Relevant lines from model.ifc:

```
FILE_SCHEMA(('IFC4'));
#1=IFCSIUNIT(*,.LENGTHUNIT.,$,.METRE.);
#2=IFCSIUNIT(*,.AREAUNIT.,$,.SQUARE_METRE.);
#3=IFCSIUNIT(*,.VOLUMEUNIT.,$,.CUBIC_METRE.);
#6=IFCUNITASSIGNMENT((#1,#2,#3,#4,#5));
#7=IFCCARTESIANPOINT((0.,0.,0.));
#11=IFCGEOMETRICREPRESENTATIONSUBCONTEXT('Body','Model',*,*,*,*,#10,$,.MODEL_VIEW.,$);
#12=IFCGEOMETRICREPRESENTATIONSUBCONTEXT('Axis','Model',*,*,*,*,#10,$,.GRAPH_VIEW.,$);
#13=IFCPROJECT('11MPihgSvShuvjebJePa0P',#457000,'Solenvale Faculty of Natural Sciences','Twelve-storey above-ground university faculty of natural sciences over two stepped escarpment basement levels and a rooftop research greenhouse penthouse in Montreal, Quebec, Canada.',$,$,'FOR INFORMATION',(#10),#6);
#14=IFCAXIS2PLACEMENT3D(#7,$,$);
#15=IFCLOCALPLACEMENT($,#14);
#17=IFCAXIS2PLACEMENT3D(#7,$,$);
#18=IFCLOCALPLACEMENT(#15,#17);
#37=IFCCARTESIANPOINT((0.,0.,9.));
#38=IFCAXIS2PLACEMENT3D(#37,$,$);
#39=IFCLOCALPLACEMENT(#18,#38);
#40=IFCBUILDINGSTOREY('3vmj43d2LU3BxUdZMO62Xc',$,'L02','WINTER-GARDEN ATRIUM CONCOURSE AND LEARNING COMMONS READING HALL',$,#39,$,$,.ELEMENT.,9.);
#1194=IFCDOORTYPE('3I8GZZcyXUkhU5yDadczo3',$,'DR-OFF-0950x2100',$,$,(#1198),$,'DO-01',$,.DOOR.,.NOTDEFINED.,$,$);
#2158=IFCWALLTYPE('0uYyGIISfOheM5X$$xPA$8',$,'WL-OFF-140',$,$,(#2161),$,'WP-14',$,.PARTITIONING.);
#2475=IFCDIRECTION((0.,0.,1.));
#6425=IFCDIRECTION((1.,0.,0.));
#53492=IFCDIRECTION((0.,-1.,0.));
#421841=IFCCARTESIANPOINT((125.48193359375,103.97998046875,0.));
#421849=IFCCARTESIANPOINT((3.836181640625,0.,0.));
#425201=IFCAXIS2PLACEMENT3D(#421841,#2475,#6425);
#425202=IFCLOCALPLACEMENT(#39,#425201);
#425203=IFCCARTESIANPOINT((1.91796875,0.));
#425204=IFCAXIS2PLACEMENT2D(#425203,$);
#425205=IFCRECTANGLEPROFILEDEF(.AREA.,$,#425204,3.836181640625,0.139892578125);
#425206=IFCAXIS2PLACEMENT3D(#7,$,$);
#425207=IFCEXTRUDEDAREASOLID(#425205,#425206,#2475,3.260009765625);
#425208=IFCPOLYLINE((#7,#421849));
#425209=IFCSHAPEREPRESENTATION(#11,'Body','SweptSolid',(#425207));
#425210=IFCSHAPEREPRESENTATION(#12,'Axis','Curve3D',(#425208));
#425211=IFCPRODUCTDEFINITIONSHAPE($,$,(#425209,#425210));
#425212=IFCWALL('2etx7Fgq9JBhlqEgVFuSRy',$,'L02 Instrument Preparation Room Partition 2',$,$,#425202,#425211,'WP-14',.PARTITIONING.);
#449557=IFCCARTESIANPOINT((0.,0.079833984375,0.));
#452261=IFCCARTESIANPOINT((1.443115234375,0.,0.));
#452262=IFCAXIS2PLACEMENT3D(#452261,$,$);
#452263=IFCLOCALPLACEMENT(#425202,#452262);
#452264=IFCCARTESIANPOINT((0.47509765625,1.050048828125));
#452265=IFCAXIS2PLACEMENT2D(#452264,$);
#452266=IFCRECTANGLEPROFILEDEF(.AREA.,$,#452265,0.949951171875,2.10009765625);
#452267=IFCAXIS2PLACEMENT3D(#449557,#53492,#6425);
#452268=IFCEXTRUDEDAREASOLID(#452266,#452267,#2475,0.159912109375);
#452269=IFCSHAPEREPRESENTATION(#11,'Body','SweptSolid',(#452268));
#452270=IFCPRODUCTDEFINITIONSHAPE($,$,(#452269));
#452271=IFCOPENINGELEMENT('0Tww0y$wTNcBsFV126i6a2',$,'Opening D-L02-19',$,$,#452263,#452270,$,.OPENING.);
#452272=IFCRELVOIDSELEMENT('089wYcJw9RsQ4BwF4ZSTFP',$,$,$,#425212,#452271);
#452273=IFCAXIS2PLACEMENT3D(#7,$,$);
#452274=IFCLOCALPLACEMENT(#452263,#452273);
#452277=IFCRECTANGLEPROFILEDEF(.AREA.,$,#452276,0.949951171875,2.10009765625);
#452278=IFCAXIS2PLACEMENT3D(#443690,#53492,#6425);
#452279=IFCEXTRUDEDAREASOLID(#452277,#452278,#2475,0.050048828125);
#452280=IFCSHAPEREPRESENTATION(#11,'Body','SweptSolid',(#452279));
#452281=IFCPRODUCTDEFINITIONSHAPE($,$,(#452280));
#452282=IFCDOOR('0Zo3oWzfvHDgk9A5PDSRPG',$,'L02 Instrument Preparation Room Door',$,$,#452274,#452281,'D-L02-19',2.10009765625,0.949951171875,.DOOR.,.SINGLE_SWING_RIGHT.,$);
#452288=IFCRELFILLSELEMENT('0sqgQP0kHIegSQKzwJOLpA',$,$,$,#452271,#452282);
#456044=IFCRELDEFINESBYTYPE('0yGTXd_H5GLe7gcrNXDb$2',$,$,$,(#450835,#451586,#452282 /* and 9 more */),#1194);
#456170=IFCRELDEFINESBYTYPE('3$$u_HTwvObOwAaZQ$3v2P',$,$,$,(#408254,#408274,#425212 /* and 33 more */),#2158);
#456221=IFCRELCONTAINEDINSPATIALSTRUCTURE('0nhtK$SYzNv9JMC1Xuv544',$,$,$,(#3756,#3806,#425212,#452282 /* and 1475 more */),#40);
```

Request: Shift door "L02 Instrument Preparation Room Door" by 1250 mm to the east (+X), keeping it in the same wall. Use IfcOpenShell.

```python
import ifcopenshell
import ifcopenshell.api.geometry
import ifcopenshell.util.placement
import ifcopenshell.util.unit

model = ifcopenshell.open("model.ifc")
unit_scale = ifcopenshell.util.unit.calculate_unit_scale(model)

door = model.by_guid("0Zo3oWzfvHDgk9A5PDSRPG")
opening = door.FillsVoids[0].RelatingOpeningElement
wall = opening.VoidsElements[0].RelatingBuildingElement

wall_matrix = ifcopenshell.util.placement.get_local_placement(wall.ObjectPlacement)
shift = wall_matrix[:3, 0] * 1.25 / unit_scale
before = ifcopenshell.util.placement.get_local_placement(door.ObjectPlacement)[:3, 3].copy()

# The door is placed relative to its opening, so it follows when the opening moves.
matrix = ifcopenshell.util.placement.get_local_placement(opening.ObjectPlacement)
matrix[:3, 3] += shift
ifcopenshell.api.geometry.edit_object_placement(
    model, product=opening, matrix=matrix, is_si=False, should_transform_children=True
)

after = ifcopenshell.util.placement.get_local_placement(door.ObjectPlacement)[:3, 3]
print("door moved by", (after - before).round(3) + 0.0)

model.write("model-out.ifc")
```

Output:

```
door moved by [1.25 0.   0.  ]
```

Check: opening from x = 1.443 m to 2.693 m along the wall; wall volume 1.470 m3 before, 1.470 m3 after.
